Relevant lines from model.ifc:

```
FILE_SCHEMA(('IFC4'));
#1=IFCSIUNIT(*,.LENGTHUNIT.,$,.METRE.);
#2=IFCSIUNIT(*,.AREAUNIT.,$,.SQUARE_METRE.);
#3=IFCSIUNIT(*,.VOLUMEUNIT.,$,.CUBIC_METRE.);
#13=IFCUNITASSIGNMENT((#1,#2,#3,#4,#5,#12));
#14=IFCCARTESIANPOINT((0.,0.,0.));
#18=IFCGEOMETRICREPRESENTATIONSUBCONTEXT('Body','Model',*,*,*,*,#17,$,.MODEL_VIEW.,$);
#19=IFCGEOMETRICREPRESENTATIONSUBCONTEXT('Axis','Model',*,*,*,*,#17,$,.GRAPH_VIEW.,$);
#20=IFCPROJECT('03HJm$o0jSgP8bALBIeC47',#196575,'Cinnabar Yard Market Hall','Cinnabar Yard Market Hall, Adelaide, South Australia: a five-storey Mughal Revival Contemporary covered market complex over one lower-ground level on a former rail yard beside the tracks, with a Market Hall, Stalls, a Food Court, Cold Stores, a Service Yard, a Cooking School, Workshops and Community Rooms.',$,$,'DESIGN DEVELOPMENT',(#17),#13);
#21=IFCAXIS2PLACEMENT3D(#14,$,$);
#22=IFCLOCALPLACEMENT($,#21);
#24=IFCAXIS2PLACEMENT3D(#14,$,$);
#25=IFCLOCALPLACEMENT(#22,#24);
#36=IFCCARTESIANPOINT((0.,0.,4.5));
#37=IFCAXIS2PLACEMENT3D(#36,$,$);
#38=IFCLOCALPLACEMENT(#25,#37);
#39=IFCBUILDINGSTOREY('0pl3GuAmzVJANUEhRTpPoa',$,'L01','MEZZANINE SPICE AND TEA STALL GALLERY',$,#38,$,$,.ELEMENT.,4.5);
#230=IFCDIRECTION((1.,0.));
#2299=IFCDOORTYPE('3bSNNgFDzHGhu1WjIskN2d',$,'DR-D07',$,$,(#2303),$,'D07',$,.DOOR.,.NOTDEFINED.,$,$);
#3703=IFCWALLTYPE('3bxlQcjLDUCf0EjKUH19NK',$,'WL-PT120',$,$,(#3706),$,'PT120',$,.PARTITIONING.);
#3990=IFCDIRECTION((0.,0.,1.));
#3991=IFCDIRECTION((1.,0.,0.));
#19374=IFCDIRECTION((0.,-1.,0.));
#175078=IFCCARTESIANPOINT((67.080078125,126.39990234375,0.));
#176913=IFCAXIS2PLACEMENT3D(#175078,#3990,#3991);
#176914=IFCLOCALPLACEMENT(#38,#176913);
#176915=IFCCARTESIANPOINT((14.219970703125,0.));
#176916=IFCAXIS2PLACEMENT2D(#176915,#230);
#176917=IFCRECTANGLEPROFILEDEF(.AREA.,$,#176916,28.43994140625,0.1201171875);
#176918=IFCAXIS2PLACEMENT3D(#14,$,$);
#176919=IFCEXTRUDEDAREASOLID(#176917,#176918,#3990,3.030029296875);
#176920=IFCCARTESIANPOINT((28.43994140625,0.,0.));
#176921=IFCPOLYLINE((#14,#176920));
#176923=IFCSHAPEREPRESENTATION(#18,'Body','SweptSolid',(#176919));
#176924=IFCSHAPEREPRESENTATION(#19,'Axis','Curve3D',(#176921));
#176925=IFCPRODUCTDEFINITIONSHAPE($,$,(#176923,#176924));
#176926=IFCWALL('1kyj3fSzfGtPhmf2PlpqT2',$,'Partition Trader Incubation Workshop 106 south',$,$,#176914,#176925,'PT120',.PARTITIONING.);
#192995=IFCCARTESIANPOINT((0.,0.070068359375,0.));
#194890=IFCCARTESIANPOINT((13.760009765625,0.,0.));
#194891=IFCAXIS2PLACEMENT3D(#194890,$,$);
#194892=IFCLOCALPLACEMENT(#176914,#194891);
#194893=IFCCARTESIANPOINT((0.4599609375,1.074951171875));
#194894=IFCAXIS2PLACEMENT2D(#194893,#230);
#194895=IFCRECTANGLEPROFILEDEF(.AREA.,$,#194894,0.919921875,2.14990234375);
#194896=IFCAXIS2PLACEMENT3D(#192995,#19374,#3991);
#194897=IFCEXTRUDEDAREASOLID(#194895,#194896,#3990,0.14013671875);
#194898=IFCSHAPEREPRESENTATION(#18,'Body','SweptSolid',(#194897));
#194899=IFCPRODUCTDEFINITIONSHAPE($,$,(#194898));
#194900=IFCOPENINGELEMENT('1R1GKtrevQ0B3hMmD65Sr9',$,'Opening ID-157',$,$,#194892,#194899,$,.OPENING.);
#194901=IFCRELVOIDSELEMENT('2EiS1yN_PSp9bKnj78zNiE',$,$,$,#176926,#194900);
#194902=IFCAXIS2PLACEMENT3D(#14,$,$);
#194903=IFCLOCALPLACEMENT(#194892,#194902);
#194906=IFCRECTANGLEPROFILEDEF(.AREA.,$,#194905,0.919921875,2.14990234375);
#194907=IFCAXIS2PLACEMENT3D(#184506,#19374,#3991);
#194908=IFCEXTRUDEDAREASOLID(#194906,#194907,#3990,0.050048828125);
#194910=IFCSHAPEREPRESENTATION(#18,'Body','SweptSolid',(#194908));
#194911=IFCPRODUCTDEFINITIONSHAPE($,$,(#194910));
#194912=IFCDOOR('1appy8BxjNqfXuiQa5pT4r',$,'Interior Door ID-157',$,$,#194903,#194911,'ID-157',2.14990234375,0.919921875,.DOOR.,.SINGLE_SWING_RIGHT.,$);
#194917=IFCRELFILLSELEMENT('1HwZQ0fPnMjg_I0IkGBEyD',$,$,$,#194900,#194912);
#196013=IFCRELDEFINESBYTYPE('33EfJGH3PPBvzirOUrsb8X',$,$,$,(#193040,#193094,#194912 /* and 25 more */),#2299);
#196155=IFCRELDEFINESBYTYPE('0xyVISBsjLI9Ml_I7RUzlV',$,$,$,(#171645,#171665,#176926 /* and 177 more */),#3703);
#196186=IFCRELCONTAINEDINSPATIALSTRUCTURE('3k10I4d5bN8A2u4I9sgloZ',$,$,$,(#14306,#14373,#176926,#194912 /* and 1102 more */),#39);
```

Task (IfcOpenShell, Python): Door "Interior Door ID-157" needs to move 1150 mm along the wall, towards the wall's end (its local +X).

```python
import ifcopenshell
import ifcopenshell.api.geometry
import ifcopenshell.util.placement
import ifcopenshell.util.unit

model = ifcopenshell.open("model.ifc")
unit_scale = ifcopenshell.util.unit.calculate_unit_scale(model)

door = model.by_id(194912)
opening = door.FillsVoids[0].RelatingOpeningElement
wall = opening.VoidsElements[0].RelatingBuildingElement

wall_matrix = ifcopenshell.util.placement.get_local_placement(wall.ObjectPlacement)
shift = wall_matrix[:3, 0] * 1.15 / unit_scale
before = ifcopenshell.util.placement.get_local_placement(door.ObjectPlacement)[:3, 3].copy()

# The door is placed relative to its opening, so it follows when the opening moves.
matrix = ifcopenshell.util.placement.get_local_placement(opening.ObjectPlacement)
matrix[:3, 3] += shift
ifcopenshell.api.geometry.edit_object_placement(
    model, product=opening, matrix=matrix, is_si=False, should_transform_children=True
)

after = ifcopenshell.util.placement.get_local_placement(door.ObjectPlacement)[:3, 3]
print("door moved by", (after - before).round(3) + 0.0)

model.write("model_edited.ifc")
```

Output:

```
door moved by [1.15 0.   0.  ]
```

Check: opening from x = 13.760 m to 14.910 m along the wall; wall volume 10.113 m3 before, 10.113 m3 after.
